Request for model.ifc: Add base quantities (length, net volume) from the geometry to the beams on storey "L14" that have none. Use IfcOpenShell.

First a look at what the model holds.

```python
import ifcopenshell
import ifcopenshell.util.element
import ifcopenshell.util.unit

model = ifcopenshell.open("model.ifc")
print(model.schema)
for unit_type in ("LENGTHUNIT", "AREAUNIT", "VOLUMEUNIT"):
    print(unit_type, ifcopenshell.util.unit.calculate_unit_scale(model, unit_type))
storey = next(s for s in model.by_type("IfcBuildingStorey") if s.Name == "L14")
beams = [e for e in ifcopenshell.util.element.get_decomposition(storey) if e.is_a("IfcBeam")]
for e in sorted(beams, key=lambda e: e.id()):
    print(e.id(), e.is_a(), e.Name, list(ifcopenshell.util.element.get_psets(e, qtos_only=True)), sep=" | ")
```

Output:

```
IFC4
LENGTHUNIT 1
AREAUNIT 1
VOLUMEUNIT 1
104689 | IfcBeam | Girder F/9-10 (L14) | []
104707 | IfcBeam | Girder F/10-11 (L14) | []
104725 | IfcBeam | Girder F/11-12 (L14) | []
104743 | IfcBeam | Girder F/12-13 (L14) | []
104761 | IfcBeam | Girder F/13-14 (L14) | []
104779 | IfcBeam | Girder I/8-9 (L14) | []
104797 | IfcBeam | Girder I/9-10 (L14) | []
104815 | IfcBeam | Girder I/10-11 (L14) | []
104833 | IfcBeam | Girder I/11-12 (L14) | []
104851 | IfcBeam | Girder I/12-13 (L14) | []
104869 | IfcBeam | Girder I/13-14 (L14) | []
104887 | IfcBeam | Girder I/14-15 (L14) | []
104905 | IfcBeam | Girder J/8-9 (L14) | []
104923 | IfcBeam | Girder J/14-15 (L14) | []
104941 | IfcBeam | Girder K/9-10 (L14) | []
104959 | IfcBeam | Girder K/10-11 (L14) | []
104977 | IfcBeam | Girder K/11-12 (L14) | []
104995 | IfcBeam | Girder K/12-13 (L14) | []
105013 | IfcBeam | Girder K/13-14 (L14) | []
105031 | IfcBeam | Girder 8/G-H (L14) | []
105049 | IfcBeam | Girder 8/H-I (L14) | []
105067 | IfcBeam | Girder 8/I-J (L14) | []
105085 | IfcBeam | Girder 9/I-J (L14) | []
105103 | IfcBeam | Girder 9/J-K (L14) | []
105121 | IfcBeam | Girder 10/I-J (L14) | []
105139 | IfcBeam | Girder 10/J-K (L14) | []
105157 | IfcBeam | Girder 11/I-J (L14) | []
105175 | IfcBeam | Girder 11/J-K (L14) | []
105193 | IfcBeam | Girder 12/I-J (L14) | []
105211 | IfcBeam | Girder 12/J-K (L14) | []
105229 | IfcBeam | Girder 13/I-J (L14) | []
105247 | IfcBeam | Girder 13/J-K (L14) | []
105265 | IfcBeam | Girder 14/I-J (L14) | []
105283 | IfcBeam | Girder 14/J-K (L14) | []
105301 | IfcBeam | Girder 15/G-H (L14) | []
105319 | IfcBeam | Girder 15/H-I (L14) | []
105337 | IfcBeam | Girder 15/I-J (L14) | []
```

```python
import ifcopenshell
import ifcopenshell.api.pset
import ifcopenshell.geom
import ifcopenshell.util.element
import ifcopenshell.util.shape
import ifcopenshell.util.unit

model = ifcopenshell.open("model.ifc")
unit_scale = ifcopenshell.util.unit.calculate_unit_scale(model)
volume_scale = ifcopenshell.util.unit.calculate_unit_scale(model, "VOLUMEUNIT")
settings = ifcopenshell.geom.settings()

storey = next(s for s in model.by_type("IfcBuildingStorey") if s.Name == "L14")
beams = [e for e in ifcopenshell.util.element.get_decomposition(storey) if e.is_a("IfcBeam")]

for e in sorted(beams, key=lambda e: e.id()):
    if ifcopenshell.util.element.get_psets(e, qtos_only=True, should_inherit=False):
        continue
    # Geometry comes back in metres, in the element's own axes.
    shape = ifcopenshell.geom.create_shape(settings, e)
    values = {
        "Length": ifcopenshell.util.shape.get_max_xyz(shape.geometry) / unit_scale,
        "NetVolume": ifcopenshell.util.shape.get_volume(shape.geometry) / volume_scale,
    }
    qto = ifcopenshell.api.pset.add_qto(model, product=e, name="Qto_BeamBaseQuantities")
    ifcopenshell.api.pset.edit_qto(model, qto=qto, properties=values)
    print(e.id(), {k: round(v, 3) for k, v in values.items()})

model.write("model_edited.ifc")
```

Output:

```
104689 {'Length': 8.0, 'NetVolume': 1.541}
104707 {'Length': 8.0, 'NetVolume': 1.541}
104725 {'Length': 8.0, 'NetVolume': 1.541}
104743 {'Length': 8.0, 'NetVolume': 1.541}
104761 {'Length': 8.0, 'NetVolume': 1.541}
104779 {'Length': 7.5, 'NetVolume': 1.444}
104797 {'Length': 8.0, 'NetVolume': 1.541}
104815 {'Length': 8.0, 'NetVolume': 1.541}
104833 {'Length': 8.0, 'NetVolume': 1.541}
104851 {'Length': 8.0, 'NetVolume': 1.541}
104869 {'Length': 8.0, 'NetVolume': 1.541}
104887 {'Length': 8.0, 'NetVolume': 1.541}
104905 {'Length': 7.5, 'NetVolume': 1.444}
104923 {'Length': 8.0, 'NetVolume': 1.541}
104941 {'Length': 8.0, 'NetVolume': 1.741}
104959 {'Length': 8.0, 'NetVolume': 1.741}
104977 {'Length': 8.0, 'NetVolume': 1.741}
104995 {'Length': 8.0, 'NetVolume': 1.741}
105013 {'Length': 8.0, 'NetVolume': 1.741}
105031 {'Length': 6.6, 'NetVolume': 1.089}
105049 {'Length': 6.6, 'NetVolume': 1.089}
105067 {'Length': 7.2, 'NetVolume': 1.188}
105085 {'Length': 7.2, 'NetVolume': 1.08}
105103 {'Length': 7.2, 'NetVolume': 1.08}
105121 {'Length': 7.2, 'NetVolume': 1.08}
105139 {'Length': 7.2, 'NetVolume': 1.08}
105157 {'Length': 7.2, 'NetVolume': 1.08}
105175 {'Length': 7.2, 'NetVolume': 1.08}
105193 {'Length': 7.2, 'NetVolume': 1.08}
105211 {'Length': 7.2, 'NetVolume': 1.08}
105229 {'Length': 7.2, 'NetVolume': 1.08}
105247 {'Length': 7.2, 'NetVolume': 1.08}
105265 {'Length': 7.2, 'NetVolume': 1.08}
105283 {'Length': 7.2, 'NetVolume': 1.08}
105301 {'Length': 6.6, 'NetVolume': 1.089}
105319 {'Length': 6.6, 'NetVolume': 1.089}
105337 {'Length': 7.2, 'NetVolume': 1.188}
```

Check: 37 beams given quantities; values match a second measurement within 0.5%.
